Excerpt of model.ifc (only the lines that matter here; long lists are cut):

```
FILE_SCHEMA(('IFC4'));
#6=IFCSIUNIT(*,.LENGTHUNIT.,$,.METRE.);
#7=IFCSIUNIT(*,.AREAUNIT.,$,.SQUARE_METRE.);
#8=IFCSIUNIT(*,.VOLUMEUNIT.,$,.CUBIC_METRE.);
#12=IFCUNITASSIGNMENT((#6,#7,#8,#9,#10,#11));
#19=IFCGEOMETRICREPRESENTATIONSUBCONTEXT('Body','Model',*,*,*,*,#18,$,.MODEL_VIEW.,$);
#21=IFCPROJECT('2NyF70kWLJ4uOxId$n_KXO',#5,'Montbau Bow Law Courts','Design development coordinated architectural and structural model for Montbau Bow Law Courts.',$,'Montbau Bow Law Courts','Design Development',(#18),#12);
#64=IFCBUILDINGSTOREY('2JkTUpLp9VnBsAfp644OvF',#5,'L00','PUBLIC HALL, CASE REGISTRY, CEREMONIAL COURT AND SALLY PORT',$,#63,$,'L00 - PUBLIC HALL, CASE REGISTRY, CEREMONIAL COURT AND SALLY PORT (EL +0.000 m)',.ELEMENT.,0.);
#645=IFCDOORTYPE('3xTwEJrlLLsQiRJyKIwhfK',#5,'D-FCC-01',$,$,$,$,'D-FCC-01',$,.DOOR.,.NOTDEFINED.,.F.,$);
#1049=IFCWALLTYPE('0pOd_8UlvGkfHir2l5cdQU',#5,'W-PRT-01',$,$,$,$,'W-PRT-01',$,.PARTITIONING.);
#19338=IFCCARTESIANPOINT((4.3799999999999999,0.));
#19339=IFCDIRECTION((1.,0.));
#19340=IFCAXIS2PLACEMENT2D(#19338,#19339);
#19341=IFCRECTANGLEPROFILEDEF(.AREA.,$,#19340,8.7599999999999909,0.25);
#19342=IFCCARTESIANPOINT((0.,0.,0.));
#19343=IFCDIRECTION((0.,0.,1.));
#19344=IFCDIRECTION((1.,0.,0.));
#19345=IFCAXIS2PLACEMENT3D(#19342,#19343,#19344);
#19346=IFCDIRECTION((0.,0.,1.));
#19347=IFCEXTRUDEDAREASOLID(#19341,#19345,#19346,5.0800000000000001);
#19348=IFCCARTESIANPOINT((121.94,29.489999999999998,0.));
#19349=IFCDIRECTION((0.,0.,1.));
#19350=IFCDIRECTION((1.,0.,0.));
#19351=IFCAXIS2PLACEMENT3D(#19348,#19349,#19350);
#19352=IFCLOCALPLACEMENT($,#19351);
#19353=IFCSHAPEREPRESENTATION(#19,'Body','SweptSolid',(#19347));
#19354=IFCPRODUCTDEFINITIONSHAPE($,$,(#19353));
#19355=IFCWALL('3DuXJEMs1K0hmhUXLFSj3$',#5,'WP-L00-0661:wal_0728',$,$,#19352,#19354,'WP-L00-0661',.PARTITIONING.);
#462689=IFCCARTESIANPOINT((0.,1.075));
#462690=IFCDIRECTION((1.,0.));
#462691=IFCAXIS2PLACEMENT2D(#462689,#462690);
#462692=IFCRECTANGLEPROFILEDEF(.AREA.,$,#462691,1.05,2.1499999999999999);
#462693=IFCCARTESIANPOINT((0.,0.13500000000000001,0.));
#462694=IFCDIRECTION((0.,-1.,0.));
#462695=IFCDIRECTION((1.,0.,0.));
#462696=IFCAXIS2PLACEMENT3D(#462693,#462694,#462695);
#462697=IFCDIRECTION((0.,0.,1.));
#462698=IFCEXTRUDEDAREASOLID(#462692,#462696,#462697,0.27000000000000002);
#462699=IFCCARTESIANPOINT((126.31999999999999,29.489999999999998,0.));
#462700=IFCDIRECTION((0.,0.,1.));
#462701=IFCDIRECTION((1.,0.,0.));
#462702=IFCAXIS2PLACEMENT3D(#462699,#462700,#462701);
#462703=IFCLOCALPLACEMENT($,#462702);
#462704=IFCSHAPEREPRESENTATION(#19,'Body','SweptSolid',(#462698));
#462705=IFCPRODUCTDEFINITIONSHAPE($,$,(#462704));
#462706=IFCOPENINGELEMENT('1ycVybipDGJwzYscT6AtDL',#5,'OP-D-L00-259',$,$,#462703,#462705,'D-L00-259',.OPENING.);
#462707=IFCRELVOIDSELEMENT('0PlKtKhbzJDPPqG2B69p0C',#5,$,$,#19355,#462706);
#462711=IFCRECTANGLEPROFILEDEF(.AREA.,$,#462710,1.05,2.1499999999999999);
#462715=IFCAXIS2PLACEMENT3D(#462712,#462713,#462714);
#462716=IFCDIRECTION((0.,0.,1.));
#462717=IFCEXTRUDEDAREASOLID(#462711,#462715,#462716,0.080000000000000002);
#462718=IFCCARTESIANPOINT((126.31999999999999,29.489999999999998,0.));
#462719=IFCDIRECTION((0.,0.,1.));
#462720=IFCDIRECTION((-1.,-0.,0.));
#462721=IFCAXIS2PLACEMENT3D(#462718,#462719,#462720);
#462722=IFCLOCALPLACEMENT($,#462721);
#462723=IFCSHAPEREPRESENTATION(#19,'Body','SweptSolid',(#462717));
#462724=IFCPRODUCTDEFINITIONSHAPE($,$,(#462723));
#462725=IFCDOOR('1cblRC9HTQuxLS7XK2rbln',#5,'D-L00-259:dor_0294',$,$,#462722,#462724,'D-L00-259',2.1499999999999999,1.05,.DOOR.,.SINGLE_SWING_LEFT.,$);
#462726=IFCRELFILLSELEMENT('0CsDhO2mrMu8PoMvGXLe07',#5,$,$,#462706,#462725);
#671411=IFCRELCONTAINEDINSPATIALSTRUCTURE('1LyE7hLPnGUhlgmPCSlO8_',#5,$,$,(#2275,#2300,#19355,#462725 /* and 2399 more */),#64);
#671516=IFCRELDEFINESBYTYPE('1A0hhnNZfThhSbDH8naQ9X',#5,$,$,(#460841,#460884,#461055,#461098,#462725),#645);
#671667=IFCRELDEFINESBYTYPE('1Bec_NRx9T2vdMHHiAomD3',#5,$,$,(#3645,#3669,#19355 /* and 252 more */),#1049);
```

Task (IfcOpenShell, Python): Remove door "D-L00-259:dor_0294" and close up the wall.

```python
import ifcopenshell
import ifcopenshell.api.feature
import ifcopenshell.api.root
import ifcopenshell.geom
import ifcopenshell.util.shape

model = ifcopenshell.open("model.ifc")
settings = ifcopenshell.geom.settings()


def volume(element):
    """Net volume in cubic metres, openings subtracted."""
    shape = ifcopenshell.geom.create_shape(settings, element)
    return ifcopenshell.util.shape.get_volume(shape.geometry)


door = model.by_guid("1cblRC9HTQuxLS7XK2rbln")
opening = door.FillsVoids[0].RelatingOpeningElement
wall = opening.VoidsElements[0].RelatingBuildingElement
before = volume(wall)

ifcopenshell.api.root.remove_product(model, product=door)
ifcopenshell.api.feature.remove_feature(model, feature=opening)

after = volume(wall)

print(f"wall volume {before:.3f} -> {after:.3f} m3")

model.write("model_updated.ifc")
```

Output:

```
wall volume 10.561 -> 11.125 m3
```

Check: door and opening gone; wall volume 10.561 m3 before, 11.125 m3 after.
